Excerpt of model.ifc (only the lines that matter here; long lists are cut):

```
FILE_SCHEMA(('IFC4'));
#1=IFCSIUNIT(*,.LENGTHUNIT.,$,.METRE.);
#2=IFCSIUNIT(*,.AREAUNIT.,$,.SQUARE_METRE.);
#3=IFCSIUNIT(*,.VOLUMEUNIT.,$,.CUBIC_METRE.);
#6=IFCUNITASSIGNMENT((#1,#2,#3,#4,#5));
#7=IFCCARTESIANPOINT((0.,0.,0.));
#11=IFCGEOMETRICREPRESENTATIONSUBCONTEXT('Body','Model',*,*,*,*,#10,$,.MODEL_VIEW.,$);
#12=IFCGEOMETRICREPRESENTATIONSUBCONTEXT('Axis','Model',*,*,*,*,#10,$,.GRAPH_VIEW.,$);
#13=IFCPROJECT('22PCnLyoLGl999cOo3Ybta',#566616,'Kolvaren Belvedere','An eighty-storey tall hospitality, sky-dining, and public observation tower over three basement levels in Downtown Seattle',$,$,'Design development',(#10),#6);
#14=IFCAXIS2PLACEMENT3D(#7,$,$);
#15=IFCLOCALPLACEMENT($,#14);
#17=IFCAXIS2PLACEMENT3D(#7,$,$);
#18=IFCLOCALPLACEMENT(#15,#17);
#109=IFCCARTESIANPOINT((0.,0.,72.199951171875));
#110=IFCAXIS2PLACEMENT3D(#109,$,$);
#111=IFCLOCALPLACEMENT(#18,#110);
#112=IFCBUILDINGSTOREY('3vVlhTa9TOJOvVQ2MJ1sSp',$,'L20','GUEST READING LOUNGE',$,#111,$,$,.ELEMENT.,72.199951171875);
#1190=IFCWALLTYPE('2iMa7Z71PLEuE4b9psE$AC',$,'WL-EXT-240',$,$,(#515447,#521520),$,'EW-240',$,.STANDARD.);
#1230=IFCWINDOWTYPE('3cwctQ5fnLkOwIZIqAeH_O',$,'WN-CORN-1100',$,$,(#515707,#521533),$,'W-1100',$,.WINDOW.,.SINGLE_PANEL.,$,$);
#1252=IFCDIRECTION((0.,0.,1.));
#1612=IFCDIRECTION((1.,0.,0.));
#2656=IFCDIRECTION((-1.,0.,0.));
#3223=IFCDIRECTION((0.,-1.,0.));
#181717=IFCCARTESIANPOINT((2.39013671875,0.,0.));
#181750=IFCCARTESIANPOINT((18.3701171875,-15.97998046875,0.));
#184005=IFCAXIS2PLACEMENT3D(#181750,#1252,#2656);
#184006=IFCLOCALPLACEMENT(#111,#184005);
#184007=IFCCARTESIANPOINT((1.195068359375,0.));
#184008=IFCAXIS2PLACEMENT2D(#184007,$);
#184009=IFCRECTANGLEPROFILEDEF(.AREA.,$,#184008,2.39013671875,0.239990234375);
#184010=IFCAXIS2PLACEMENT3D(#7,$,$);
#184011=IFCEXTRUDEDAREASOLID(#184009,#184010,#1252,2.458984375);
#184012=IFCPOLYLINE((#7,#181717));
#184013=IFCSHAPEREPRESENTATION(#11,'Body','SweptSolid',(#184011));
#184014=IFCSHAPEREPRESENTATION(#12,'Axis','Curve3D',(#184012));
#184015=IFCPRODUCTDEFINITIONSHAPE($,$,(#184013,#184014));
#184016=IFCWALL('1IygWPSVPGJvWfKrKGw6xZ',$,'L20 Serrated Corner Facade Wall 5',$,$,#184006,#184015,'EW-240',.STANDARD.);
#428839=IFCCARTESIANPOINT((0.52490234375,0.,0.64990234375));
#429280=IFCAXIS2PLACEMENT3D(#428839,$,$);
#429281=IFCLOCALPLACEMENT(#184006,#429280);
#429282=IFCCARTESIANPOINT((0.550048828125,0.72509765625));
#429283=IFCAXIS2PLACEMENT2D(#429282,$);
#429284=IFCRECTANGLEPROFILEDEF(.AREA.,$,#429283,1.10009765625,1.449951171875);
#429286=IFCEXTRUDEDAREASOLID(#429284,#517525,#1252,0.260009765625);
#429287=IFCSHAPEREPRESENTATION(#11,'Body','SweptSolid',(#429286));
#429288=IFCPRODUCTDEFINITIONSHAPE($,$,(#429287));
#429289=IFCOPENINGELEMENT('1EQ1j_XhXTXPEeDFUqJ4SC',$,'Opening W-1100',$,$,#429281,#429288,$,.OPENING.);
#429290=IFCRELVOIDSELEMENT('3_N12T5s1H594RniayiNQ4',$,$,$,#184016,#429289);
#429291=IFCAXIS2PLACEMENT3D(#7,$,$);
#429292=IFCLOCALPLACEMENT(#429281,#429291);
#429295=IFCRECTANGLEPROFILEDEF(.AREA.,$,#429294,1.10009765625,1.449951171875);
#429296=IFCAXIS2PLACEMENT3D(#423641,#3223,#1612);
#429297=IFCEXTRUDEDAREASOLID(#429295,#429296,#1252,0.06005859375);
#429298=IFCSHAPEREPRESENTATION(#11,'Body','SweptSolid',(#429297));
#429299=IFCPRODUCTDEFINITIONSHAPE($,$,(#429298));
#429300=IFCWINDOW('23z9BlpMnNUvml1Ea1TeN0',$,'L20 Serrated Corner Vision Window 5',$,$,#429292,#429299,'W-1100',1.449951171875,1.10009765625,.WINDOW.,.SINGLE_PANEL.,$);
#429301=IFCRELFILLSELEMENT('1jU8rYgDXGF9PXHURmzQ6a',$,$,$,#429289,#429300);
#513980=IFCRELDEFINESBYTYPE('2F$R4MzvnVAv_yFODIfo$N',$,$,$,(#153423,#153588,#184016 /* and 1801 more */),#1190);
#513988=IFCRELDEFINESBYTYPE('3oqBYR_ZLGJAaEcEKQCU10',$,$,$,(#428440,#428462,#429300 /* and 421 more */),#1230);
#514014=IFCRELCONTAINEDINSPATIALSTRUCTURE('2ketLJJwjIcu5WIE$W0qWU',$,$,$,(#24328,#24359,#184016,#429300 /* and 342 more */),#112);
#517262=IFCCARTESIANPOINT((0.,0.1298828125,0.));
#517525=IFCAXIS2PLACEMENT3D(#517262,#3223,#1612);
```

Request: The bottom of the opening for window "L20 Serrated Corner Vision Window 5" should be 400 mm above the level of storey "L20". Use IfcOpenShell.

```python
import numpy as np
import ifcopenshell
import ifcopenshell.api.geometry
import ifcopenshell.geom
import ifcopenshell.util.element
import ifcopenshell.util.placement
import ifcopenshell.util.shape
import ifcopenshell.util.unit

model = ifcopenshell.open("model.ifc")
unit_scale = ifcopenshell.util.unit.calculate_unit_scale(model)

window = model.by_guid("23z9BlpMnNUvml1Ea1TeN0")
opening = window.FillsVoids[0].RelatingOpeningElement
storey = ifcopenshell.util.element.get_container(window, ifc_class="IfcBuildingStorey")
level = ifcopenshell.util.placement.get_local_placement(storey.ObjectPlacement)[2, 3]

# The opening's origin need not be at the sill, so measure its lowest point.
shape = ifcopenshell.geom.create_shape(ifcopenshell.geom.settings(), opening)
bottom = ifcopenshell.util.shape.get_shape_bottom_elevation(shape, shape.geometry) / unit_scale
dz = level + 0.4 / unit_scale - bottom

shift = np.array([0.0, 0.0, dz])
# The window is placed relative to its opening, so it follows when the opening moves.
matrix = ifcopenshell.util.placement.get_local_placement(opening.ObjectPlacement)
matrix[:3, 3] += shift
ifcopenshell.api.geometry.edit_object_placement(
    model, product=opening, matrix=matrix, is_si=False, should_transform_children=True
)

print(f"moved by {dz * unit_scale:+.3f} m")

model.write("model_rev.ifc")
```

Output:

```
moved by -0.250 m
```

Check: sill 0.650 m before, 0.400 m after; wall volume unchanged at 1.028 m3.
